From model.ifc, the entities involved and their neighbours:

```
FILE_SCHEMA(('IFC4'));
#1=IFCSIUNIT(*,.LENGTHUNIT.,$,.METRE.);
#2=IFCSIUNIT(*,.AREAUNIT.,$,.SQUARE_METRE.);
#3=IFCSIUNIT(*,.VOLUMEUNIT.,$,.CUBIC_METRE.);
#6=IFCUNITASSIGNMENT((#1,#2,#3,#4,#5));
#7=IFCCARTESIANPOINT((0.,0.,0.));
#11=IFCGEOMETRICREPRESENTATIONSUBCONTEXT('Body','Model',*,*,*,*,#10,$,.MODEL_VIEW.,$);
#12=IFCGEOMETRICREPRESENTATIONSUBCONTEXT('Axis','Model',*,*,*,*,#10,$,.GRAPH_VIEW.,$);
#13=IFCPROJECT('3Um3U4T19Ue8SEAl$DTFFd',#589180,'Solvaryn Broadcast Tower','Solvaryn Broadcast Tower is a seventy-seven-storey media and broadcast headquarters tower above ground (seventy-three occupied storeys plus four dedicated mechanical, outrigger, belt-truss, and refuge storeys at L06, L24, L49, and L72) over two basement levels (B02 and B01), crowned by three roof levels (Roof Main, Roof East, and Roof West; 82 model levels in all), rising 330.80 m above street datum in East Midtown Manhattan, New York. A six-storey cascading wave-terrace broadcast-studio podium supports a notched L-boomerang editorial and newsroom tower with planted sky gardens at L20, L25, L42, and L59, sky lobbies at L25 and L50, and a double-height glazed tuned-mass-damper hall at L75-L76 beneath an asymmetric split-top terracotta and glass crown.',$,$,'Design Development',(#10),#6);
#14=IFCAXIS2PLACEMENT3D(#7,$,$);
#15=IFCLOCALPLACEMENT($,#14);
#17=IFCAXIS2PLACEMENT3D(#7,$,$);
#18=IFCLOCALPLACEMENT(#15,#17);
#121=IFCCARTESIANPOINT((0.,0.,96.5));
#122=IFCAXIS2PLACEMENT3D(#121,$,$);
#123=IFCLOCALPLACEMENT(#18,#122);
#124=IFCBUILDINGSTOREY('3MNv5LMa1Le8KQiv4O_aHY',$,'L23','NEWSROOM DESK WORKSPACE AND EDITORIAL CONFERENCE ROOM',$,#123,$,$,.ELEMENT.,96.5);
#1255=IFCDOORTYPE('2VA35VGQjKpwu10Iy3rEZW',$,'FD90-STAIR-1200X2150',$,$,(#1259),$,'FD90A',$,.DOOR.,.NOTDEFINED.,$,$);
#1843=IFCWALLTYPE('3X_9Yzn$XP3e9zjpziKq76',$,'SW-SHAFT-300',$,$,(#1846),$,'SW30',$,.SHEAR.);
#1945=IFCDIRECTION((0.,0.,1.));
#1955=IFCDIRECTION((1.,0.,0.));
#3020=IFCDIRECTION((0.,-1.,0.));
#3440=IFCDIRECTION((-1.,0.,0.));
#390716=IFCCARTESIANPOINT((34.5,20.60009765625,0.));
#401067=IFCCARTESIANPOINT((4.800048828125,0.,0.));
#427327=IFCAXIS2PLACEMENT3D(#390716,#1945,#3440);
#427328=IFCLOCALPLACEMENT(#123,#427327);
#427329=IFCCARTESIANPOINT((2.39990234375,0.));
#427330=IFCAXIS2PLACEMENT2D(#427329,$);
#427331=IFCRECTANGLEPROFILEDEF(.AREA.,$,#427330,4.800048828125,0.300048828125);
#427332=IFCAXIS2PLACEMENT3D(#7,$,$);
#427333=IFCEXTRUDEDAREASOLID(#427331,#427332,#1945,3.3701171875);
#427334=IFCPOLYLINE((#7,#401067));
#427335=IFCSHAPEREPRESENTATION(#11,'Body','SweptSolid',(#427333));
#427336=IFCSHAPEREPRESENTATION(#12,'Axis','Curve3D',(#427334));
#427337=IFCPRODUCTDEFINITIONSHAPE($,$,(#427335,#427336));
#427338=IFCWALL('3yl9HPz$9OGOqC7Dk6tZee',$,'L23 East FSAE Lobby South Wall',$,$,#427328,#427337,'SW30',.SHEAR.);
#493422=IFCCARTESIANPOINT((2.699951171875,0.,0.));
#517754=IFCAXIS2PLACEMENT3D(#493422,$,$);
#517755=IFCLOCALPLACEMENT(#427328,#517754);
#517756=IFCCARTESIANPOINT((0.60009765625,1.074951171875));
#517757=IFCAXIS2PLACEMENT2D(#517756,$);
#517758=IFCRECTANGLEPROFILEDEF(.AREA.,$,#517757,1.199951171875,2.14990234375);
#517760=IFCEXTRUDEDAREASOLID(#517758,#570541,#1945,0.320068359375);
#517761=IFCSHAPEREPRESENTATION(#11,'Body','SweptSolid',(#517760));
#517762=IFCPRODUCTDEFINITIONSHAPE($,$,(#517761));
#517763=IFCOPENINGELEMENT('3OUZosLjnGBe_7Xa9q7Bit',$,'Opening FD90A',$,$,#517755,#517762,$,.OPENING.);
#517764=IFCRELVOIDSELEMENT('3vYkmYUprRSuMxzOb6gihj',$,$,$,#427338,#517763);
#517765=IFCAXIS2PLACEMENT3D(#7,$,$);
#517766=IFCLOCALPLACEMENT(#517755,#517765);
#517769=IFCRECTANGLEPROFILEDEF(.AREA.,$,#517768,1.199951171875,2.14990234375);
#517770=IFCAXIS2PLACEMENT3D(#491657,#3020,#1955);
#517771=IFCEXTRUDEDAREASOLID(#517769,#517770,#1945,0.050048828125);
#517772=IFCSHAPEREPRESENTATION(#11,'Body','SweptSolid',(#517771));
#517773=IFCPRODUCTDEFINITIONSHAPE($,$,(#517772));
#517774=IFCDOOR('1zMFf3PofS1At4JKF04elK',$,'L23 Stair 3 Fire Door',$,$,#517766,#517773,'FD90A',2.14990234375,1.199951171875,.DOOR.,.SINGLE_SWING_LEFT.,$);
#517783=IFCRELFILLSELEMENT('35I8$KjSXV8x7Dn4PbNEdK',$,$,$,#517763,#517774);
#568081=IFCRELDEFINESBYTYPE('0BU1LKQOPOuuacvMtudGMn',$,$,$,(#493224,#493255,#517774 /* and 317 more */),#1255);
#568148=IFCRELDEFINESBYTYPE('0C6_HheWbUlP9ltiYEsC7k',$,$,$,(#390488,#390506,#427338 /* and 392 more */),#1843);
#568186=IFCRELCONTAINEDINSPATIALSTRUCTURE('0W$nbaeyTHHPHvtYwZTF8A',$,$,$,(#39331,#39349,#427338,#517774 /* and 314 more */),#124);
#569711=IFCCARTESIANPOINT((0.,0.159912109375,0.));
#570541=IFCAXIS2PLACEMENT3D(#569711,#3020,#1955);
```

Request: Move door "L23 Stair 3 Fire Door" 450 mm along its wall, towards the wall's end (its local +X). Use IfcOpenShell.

```python
import ifcopenshell
import ifcopenshell.api.geometry
import ifcopenshell.util.placement

model = ifcopenshell.open("model.ifc")

door = model.by_guid("1zMFf3PofS1At4JKF04elK")
opening = door.FillsVoids[0].RelatingOpeningElement
wall = opening.VoidsElements[0].RelatingBuildingElement

wall_matrix = ifcopenshell.util.placement.get_local_placement(wall.ObjectPlacement)
shift = wall_matrix[:3, 0] * 0.45
before = ifcopenshell.util.placement.get_local_placement(door.ObjectPlacement)[:3, 3].copy()

# The door is placed relative to its opening, so it follows when the opening moves.
matrix = ifcopenshell.util.placement.get_local_placement(opening.ObjectPlacement)
matrix[:3, 3] += shift
ifcopenshell.api.geometry.edit_object_placement(
    model, product=opening, matrix=matrix, is_si=False, should_transform_children=True
)

after = ifcopenshell.util.placement.get_local_placement(door.ObjectPlacement)[:3, 3]
print("door moved by", (after - before).round(3) + 0.0)

model.write("model_rev.ifc")
```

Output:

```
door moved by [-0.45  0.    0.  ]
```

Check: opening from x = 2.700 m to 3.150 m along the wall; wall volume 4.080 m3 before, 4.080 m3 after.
